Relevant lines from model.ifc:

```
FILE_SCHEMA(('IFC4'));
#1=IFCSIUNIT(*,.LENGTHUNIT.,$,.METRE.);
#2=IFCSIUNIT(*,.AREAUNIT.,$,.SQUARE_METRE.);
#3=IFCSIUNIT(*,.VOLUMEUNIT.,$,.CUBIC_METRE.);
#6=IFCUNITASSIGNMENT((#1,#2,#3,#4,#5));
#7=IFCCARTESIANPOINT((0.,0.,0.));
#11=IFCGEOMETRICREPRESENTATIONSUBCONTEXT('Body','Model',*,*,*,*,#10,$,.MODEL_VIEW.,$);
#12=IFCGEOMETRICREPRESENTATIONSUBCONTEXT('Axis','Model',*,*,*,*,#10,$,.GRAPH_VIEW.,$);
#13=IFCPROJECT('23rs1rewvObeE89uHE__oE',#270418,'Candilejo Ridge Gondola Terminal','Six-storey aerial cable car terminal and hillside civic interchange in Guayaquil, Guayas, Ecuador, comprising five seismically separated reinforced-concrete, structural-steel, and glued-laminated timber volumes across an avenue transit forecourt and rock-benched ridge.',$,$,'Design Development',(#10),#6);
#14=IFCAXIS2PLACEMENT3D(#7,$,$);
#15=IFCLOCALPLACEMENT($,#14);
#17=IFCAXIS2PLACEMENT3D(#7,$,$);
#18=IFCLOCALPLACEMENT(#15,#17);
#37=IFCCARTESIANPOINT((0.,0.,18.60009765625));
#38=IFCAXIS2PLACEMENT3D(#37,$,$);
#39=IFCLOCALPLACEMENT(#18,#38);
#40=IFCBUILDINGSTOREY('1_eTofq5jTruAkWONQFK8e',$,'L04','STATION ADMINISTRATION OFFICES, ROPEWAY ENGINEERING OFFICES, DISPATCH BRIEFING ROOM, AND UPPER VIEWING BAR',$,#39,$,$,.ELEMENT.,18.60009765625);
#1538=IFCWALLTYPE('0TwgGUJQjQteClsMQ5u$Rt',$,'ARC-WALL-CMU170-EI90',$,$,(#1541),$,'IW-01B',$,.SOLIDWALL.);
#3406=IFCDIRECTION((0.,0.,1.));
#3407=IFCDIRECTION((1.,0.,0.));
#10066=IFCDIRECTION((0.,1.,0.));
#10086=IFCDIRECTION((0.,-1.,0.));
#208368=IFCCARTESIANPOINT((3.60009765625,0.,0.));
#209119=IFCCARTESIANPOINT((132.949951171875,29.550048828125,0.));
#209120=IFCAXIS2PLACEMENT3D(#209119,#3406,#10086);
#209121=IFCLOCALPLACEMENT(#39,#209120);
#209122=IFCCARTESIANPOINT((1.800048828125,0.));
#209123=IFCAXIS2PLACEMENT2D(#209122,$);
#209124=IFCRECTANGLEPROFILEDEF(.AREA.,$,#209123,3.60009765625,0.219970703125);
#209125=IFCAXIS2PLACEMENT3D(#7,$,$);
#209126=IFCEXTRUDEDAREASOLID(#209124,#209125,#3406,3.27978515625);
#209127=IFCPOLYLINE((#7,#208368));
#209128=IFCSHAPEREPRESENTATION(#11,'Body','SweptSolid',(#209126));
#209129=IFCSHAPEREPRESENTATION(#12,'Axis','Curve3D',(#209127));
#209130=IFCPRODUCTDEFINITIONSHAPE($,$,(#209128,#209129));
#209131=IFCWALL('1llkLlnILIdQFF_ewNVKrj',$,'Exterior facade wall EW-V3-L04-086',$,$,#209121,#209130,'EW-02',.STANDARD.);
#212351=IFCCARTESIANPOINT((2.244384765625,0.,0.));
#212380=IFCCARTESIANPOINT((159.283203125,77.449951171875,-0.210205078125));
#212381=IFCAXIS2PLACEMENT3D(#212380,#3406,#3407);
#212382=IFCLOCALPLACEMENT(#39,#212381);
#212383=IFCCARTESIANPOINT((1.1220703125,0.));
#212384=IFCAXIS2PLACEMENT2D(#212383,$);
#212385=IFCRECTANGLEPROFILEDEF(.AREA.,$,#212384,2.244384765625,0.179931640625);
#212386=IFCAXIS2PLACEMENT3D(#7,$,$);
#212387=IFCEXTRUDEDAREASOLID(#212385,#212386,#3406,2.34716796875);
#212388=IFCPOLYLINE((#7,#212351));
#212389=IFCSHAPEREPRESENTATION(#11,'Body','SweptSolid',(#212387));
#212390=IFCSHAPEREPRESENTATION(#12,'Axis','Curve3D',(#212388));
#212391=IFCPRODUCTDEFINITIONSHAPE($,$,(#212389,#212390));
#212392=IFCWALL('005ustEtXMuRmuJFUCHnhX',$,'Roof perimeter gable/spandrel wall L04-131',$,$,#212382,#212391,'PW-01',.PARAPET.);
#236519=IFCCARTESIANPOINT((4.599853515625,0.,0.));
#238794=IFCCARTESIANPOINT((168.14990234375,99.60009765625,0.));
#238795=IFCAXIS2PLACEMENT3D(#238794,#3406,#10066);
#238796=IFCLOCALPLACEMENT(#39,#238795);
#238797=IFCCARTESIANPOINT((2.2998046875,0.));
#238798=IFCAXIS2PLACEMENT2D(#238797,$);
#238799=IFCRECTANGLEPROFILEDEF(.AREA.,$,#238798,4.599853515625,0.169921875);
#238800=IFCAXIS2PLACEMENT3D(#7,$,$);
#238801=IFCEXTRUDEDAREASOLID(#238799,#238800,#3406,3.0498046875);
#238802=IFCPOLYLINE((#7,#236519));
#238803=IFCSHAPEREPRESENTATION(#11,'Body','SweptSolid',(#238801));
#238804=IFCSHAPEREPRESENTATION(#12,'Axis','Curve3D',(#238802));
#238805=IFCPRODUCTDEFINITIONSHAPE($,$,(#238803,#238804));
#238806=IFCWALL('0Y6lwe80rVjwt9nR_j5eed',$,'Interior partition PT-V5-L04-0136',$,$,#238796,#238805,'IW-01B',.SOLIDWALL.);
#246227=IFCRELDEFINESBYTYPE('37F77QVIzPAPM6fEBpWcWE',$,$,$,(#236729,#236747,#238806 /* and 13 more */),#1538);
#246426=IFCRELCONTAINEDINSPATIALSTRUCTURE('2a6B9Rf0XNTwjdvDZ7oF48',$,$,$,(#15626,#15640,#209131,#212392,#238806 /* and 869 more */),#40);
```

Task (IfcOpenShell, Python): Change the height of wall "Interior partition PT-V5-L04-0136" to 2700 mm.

```python
import ifcopenshell
import ifcopenshell.geom
import ifcopenshell.util.representation
import ifcopenshell.util.shape
import ifcopenshell.util.unit

model = ifcopenshell.open("model.ifc")
unit_scale = ifcopenshell.util.unit.calculate_unit_scale(model)
settings = ifcopenshell.geom.settings()


def volume(element):
    """Net volume in cubic metres, openings subtracted."""
    shape = ifcopenshell.geom.create_shape(settings, element)
    return ifcopenshell.util.shape.get_volume(shape.geometry)


wall = model.by_guid("0Y6lwe80rVjwt9nR_j5eed")
before = volume(wall)

body = ifcopenshell.util.representation.get_representation(wall, "Model", "Body")
solid = body.Items[0]
old_height = solid.Depth
solid.Depth = 2.7 / unit_scale
after = volume(wall)

print(f"height {old_height:g} -> {solid.Depth:g}, volume {before:.3f} -> {after:.3f} m3")

model.write("model-out.ifc")
```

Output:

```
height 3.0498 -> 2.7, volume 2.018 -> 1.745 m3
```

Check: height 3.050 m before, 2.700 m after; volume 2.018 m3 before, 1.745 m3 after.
